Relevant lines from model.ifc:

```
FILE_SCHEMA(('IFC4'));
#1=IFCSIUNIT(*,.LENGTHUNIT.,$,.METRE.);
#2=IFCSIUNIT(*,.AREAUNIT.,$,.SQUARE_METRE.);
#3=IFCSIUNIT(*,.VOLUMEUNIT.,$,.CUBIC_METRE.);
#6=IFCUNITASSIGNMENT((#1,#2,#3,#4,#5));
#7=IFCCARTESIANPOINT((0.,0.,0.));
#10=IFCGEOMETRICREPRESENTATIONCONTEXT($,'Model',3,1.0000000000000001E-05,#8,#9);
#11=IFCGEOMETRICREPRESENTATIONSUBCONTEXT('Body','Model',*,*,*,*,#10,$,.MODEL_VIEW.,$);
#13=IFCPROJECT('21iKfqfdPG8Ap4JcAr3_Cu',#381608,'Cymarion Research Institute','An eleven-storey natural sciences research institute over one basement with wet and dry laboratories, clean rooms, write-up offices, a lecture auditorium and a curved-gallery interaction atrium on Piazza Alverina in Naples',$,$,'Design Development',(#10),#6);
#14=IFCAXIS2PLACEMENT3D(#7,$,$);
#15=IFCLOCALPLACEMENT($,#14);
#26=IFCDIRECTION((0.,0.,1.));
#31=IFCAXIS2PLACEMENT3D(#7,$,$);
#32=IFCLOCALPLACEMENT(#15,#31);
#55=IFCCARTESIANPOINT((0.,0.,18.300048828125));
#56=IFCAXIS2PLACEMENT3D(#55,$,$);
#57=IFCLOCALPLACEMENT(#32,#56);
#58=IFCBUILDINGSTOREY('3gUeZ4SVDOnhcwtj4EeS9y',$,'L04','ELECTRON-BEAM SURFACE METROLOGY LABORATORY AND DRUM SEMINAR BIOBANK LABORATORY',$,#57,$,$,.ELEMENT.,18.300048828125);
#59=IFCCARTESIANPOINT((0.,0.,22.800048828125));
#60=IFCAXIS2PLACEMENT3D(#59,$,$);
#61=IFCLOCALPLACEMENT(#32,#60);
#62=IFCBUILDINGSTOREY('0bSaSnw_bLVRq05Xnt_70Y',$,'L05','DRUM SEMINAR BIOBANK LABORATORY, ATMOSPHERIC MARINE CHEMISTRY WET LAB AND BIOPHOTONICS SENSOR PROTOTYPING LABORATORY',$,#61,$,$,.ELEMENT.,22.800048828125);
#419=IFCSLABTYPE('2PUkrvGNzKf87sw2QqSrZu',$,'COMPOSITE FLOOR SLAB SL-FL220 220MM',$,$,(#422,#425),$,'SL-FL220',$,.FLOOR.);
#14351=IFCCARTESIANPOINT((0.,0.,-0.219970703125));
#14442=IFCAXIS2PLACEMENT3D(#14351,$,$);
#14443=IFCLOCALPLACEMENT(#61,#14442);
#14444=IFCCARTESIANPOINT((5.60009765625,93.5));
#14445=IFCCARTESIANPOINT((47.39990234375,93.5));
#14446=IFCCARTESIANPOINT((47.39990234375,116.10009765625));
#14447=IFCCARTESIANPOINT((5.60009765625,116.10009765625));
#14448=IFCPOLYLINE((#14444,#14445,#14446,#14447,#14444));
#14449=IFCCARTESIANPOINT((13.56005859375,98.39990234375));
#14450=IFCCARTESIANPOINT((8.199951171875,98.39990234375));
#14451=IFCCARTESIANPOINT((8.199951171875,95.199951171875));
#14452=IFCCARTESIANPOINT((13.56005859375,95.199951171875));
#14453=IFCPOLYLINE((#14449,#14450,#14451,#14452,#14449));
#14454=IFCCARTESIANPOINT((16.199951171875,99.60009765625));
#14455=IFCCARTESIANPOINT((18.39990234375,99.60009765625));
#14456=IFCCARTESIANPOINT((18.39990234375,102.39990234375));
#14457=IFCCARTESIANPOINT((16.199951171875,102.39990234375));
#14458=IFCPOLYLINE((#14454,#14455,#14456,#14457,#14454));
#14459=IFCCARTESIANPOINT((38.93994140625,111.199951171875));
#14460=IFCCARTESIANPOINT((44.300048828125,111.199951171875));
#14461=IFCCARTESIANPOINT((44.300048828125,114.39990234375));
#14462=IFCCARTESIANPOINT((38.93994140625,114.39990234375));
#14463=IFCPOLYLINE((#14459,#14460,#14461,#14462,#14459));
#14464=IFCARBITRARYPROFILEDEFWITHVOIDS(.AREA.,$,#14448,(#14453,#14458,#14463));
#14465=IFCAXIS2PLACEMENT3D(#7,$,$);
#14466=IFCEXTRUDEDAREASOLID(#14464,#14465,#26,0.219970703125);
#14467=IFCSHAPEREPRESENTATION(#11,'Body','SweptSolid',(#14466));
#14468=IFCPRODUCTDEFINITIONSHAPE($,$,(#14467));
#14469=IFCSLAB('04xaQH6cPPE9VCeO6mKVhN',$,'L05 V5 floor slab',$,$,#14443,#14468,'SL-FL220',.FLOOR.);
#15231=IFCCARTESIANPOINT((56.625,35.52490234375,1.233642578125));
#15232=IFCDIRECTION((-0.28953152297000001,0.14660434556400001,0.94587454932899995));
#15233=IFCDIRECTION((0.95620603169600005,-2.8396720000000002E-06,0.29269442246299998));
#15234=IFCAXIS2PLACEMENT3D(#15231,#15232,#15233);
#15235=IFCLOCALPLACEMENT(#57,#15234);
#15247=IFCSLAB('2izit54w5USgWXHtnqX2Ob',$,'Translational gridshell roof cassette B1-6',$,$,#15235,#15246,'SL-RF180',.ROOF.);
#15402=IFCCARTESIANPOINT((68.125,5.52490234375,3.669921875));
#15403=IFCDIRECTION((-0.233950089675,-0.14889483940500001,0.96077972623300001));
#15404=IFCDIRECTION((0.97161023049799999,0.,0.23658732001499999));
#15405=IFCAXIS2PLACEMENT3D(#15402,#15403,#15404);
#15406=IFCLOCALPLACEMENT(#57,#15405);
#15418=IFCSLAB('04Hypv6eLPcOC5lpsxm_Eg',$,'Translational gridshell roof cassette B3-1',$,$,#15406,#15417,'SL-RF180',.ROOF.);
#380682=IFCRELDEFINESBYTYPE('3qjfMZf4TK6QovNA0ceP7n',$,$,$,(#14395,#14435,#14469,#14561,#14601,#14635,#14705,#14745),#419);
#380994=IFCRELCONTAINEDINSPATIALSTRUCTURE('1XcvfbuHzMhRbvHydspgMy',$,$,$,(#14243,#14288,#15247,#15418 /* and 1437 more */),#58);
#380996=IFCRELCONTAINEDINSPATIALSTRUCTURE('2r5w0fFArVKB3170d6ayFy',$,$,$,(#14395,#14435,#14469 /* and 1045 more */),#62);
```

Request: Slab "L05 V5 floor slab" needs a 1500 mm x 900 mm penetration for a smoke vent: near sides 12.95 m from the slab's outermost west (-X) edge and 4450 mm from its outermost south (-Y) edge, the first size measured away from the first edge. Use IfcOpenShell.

```python
import numpy as np
import ifcopenshell
import ifcopenshell.api.feature
import ifcopenshell.api.geometry
import ifcopenshell.api.root
import ifcopenshell.geom
import ifcopenshell.util.placement
import ifcopenshell.util.representation
import ifcopenshell.util.shape
import ifcopenshell.util.unit

model = ifcopenshell.open("model.ifc")
unit_scale = ifcopenshell.util.unit.calculate_unit_scale(model)
settings = ifcopenshell.geom.settings()


def volume(element):
    """Net volume in cubic metres, openings subtracted."""
    shape = ifcopenshell.geom.create_shape(settings, element)
    return ifcopenshell.util.shape.get_volume(shape.geometry)


slab = model.by_guid("04xaQH6cPPE9VCeO6mKVhN")
before = volume(slab)

# Extent in the slab's own axes, in metres. The edges named are its -X and -Y sides.
slab_shape = ifcopenshell.geom.create_shape(settings, slab)
vertices = ifcopenshell.util.shape.get_vertices(slab_shape.geometry)
x_min, y_min, bottom = vertices.min(axis=0)
top = vertices[:, 2].max()

opening = ifcopenshell.api.root.create_entity(model, ifc_class="IfcOpeningElement", name="Smoke vent opening", predefined_type="OPENING")
context = ifcopenshell.util.representation.get_context(model, "Model", "Body", "MODEL_VIEW")
width, depth = 1.5, 0.9
outline = [(0.0, 0.0), (width, 0.0), (width, depth), (0.0, depth), (0.0, 0.0)]
# Overshoot both faces by 50 mm so the cut is clean.
shape = ifcopenshell.api.geometry.add_slab_representation(
    model, context=context, depth=top - bottom + 0.1, polyline=outline
)
ifcopenshell.api.geometry.assign_representation(model, product=opening, representation=shape)

matrix = ifcopenshell.util.placement.get_local_placement(slab.ObjectPlacement)
matrix[:, 3] = matrix @ np.append(np.array([x_min + 12.95, y_min + 4.45, bottom - 0.05]) / unit_scale, 1.0)
ifcopenshell.api.geometry.edit_object_placement(model, product=opening, matrix=matrix, is_si=False)
ifcopenshell.api.feature.add_feature(model, feature=opening, element=slab)

after = volume(slab)

print(f"slab volume {before:.3f} -> {after:.3f} m3")

model.write("model_updated.ifc")
```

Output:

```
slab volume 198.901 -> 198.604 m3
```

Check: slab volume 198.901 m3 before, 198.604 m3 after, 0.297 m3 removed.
